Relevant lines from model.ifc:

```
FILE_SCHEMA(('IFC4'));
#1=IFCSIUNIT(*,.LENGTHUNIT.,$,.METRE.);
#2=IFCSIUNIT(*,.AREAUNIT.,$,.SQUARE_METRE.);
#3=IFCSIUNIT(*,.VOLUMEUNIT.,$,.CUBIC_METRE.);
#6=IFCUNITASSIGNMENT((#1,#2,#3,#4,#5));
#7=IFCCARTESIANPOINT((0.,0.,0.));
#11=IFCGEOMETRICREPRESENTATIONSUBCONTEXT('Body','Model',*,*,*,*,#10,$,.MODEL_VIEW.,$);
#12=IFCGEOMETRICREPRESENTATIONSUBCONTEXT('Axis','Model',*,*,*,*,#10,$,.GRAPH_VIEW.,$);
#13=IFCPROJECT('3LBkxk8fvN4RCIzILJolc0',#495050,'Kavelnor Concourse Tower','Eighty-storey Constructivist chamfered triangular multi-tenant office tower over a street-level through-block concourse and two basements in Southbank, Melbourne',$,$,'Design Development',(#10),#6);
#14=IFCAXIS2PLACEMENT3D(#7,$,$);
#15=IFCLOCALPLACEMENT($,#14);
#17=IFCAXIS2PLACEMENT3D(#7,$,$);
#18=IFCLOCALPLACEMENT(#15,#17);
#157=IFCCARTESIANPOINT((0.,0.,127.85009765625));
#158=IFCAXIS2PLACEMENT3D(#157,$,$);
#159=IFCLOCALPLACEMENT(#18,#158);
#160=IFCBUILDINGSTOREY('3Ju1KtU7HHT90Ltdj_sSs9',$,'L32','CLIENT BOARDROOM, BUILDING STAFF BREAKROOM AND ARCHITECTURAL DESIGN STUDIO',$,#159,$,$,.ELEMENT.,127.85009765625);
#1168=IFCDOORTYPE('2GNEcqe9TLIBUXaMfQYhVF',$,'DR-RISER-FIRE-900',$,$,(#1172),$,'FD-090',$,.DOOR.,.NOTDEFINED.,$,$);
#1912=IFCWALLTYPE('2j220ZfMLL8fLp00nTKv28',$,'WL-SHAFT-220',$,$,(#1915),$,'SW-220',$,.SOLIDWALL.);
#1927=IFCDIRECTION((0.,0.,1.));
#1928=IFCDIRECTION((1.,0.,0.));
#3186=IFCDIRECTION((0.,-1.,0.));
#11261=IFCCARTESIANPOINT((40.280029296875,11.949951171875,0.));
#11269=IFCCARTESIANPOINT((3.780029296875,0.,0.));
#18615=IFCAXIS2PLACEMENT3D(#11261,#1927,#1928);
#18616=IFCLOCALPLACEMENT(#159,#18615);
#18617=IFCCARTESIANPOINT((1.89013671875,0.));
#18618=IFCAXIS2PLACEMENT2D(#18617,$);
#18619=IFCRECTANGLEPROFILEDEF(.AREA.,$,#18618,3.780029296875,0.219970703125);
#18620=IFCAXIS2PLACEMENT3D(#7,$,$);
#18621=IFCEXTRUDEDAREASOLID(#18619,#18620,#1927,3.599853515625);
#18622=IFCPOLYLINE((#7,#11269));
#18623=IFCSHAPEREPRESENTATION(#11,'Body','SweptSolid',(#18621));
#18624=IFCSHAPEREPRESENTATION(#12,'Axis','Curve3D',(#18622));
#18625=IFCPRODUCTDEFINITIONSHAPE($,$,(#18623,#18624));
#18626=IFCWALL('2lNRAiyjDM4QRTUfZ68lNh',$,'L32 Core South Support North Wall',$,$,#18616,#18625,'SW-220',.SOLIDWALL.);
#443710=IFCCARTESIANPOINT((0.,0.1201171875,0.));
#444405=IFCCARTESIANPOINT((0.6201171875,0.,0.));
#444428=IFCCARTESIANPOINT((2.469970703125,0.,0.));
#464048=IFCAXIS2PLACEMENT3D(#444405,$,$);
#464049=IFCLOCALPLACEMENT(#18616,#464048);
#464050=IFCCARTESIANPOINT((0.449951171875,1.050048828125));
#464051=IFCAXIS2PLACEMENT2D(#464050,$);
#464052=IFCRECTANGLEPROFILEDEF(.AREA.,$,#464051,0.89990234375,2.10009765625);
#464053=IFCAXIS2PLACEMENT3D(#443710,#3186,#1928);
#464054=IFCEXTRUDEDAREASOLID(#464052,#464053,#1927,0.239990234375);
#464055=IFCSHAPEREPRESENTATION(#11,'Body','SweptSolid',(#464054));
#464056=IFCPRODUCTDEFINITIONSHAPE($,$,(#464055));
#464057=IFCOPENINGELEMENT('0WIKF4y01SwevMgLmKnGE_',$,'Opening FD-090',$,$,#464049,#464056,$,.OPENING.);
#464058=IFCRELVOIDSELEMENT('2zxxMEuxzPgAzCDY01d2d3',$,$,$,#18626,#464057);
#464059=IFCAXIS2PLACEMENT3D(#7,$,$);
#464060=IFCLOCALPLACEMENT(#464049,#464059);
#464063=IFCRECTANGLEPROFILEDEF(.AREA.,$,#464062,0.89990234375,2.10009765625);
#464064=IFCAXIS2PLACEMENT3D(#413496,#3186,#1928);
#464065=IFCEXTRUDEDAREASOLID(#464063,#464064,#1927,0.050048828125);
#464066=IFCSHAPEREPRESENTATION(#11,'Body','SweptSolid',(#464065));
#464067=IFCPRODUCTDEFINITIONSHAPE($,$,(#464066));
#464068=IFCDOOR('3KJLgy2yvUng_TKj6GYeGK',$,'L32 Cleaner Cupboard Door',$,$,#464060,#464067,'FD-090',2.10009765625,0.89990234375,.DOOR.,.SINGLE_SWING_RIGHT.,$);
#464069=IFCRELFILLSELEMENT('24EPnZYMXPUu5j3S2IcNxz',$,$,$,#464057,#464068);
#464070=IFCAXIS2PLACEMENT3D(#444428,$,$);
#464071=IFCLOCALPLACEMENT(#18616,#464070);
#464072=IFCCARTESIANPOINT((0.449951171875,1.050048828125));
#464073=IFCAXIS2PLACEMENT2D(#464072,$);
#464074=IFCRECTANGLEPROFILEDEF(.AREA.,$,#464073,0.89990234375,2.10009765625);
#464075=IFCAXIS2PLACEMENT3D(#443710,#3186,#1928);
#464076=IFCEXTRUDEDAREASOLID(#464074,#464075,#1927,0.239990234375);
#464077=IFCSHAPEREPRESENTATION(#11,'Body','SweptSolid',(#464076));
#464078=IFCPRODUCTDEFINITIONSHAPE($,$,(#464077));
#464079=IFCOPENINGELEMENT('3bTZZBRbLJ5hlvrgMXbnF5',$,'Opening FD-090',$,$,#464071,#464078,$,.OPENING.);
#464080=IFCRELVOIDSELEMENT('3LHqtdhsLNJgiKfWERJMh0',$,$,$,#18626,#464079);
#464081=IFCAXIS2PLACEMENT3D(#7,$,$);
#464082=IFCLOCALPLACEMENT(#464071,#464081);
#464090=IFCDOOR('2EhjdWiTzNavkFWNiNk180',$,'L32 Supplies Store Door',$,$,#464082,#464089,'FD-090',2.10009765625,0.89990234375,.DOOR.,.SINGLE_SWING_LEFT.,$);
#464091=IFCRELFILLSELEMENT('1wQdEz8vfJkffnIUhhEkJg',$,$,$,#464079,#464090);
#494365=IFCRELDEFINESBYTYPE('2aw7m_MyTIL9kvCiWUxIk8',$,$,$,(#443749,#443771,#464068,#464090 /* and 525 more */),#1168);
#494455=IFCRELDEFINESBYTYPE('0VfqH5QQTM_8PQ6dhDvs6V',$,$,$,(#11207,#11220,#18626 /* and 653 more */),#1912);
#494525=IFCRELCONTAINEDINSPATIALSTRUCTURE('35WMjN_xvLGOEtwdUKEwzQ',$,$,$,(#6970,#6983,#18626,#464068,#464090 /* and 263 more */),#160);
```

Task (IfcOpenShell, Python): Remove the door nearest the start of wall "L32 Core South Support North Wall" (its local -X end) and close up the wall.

```python
import ifcopenshell
import ifcopenshell.api.feature
import ifcopenshell.api.root
import ifcopenshell.geom
import ifcopenshell.util.shape

model = ifcopenshell.open("model.ifc")
settings = ifcopenshell.geom.settings()


def volume(element):
    """Net volume in cubic metres, openings subtracted."""
    shape = ifcopenshell.geom.create_shape(settings, element)
    return ifcopenshell.util.shape.get_volume(shape.geometry)


door = model.by_guid("3KJLgy2yvUng_TKj6GYeGK")
opening = door.FillsVoids[0].RelatingOpeningElement
wall = opening.VoidsElements[0].RelatingBuildingElement
before = volume(wall)

ifcopenshell.api.root.remove_product(model, product=door)
ifcopenshell.api.feature.remove_feature(model, feature=opening)

after = volume(wall)

print(f"wall volume {before:.3f} -> {after:.3f} m3")

model.write("model_v2.ifc")
```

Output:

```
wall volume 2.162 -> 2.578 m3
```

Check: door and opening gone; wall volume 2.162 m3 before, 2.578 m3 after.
